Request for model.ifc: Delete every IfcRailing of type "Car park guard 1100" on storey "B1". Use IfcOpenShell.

First a look at what the model holds.

```python
import ifcopenshell
import ifcopenshell.util.element

model = ifcopenshell.open("model.ifc")
print(model.schema)
storey = next(s for s in model.by_type("IfcBuildingStorey") if s.Name == "B1")
railings = [e for e in ifcopenshell.util.element.get_decomposition(storey) if e.is_a("IfcRailing")]
seen = {}
for e in railings:
    element_type = ifcopenshell.util.element.get_type(e)
    name = element_type.Name if element_type not in (None, e) else None
    seen[name] = seen.get(name, 0) + 1
for name, count in sorted(seen.items(), key=str):
    print(count, "x", name)
```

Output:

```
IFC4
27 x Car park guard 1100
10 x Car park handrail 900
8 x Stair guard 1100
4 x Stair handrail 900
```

```python
import ifcopenshell
import ifcopenshell.api.root
import ifcopenshell.util.element

model = ifcopenshell.open("model.ifc")

storey = next(s for s in model.by_type("IfcBuildingStorey") if s.Name == "B1")
railings = [e for e in ifcopenshell.util.element.get_decomposition(storey) if e.is_a("IfcRailing")]
targets = [e for e in railings if (t := ifcopenshell.util.element.get_type(e)) not in (None, e) and t.Name == "Car park guard 1100"]

for e in targets:
    ifcopenshell.api.root.remove_product(model, product=e)
print(len(targets), "removed")

model.write("model_edited.ifc")
```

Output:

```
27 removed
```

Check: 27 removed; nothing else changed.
